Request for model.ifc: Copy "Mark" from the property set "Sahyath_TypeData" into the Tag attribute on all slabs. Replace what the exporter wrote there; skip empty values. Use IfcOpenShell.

First a look at what the model holds.

```python
import ifcopenshell
import ifcopenshell.util.element

model = ifcopenshell.open("model.ifc")
print(model.schema)
slabs = model.by_type("IfcSlab")
print(len(slabs), "slabs")
for e in slabs[:8]:
    source = ifcopenshell.util.element.get_pset(e, "Sahyath_TypeData", "Mark")
    target = e.Tag
    print(e.id(), repr(source), repr(target), sep=" | ")
```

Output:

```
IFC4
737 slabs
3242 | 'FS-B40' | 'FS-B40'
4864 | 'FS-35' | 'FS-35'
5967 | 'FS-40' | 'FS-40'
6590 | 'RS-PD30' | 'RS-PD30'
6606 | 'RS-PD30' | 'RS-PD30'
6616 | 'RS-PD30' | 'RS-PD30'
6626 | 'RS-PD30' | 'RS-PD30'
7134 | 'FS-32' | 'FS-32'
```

```python
import ifcopenshell
import ifcopenshell.util.element

model = ifcopenshell.open("model.ifc")

count = 0
for e in model.by_type("IfcSlab"):
    value = ifcopenshell.util.element.get_pset(e, "Sahyath_TypeData", "Mark")
    current = e.Tag
    if not value or not value.strip() or current == value:
        continue
    e.Tag = value
    count += 1

print(count, "slabs updated")

model.write("model_rev.ifc")
```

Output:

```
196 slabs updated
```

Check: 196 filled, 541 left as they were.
